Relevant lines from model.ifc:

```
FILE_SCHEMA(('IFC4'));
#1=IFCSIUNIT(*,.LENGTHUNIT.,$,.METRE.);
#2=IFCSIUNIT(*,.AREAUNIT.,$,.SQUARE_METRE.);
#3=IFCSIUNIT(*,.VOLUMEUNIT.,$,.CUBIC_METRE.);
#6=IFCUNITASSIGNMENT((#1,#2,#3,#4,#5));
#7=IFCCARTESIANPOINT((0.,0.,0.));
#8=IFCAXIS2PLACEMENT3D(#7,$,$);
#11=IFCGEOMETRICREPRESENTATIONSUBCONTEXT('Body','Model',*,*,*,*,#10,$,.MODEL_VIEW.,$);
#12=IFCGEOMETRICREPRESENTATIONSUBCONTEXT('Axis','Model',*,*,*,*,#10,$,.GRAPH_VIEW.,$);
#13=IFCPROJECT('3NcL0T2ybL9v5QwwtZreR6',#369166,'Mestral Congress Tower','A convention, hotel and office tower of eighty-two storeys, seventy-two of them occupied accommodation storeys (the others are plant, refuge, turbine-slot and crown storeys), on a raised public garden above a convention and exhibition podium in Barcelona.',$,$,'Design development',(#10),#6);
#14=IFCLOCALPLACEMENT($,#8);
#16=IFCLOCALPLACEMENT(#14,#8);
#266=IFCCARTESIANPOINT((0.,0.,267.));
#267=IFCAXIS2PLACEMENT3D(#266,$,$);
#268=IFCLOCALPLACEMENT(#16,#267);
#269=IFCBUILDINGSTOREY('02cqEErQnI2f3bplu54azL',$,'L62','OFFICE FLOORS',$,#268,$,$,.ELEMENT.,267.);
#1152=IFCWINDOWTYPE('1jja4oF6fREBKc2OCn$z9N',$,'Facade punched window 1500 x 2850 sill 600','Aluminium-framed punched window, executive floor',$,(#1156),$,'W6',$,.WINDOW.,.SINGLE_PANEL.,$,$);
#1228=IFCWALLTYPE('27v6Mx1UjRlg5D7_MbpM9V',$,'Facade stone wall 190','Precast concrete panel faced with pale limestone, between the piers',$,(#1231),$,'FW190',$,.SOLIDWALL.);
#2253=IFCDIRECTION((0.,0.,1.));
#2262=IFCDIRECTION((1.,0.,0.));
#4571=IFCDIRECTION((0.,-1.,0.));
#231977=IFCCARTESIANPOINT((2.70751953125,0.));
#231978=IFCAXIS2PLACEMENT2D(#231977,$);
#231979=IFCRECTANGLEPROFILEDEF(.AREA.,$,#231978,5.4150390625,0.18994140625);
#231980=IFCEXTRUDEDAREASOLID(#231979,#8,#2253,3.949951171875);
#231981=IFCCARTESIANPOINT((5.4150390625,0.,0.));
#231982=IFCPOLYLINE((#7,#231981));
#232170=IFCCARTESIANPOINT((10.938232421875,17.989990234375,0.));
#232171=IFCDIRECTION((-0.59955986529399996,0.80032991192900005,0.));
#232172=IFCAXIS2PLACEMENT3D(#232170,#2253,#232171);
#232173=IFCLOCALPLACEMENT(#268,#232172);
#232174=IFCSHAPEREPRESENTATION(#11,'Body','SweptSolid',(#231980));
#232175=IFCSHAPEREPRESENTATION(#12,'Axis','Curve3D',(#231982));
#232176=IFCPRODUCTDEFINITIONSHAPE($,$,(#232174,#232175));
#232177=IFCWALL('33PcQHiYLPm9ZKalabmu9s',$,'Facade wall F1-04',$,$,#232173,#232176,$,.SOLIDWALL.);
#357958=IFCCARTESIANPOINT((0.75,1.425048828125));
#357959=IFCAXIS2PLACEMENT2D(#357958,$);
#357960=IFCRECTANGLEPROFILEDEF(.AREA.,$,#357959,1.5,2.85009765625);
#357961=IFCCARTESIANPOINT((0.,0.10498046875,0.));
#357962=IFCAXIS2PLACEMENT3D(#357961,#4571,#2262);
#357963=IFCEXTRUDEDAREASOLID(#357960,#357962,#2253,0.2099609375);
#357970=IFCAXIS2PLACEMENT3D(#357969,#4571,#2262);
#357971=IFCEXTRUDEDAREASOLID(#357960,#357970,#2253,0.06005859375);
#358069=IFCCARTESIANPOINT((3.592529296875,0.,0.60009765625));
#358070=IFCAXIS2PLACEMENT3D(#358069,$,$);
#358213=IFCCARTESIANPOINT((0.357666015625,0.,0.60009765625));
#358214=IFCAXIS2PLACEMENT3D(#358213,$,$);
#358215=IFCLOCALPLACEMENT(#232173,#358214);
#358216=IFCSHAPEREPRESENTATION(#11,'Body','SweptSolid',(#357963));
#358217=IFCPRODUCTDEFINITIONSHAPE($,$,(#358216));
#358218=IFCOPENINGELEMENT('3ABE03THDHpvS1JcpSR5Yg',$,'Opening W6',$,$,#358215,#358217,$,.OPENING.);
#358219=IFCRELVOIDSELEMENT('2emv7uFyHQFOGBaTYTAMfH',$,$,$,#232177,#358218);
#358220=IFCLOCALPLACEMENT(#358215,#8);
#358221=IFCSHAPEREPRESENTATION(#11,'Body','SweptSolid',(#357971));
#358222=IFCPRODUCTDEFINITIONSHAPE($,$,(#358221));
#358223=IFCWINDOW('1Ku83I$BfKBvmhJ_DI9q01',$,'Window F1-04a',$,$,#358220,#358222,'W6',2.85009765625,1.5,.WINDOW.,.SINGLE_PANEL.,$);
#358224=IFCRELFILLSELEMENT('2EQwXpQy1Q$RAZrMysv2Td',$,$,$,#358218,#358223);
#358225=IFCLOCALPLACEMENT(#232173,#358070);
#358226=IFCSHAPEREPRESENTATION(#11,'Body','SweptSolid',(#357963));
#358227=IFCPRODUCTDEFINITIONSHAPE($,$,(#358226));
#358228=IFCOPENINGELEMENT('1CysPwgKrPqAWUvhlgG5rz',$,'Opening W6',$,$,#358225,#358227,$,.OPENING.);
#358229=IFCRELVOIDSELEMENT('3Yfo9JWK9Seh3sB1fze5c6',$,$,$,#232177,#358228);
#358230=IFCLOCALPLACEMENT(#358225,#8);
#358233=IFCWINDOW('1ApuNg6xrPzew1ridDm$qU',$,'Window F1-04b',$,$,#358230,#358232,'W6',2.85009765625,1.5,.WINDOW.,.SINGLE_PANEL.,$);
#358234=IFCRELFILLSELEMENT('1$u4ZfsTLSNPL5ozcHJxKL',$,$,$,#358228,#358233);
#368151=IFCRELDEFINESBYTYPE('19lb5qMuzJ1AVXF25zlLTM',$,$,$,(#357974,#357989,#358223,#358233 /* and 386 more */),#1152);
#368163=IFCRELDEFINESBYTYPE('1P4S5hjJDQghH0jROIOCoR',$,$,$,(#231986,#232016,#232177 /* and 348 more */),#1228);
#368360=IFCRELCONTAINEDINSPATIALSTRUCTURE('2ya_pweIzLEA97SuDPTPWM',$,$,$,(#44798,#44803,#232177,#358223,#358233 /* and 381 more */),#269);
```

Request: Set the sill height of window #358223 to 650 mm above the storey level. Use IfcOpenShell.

```python
import numpy as np
import ifcopenshell
import ifcopenshell.api.geometry
import ifcopenshell.geom
import ifcopenshell.util.element
import ifcopenshell.util.placement
import ifcopenshell.util.shape
import ifcopenshell.util.unit

model = ifcopenshell.open("model.ifc")
unit_scale = ifcopenshell.util.unit.calculate_unit_scale(model)

window = model.by_guid("1Ku83I$BfKBvmhJ_DI9q01")
opening = window.FillsVoids[0].RelatingOpeningElement
storey = ifcopenshell.util.element.get_container(window, ifc_class="IfcBuildingStorey")
level = ifcopenshell.util.placement.get_local_placement(storey.ObjectPlacement)[2, 3]

# The opening's origin need not be at the sill, so measure its lowest point.
shape = ifcopenshell.geom.create_shape(ifcopenshell.geom.settings(), opening)
bottom = ifcopenshell.util.shape.get_shape_bottom_elevation(shape, shape.geometry) / unit_scale
dz = level + 0.65 - bottom

shift = np.array([0.0, 0.0, dz])
# The window is placed relative to its opening, so it follows when the opening moves.
matrix = ifcopenshell.util.placement.get_local_placement(opening.ObjectPlacement)
matrix[:3, 3] += shift
ifcopenshell.api.geometry.edit_object_placement(
    model, product=opening, matrix=matrix, is_si=False, should_transform_children=True
)

print(f"moved by {dz * unit_scale:+.3f} m")

model.write("model-out.ifc")
```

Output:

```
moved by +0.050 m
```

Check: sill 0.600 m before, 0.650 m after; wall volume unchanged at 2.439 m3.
